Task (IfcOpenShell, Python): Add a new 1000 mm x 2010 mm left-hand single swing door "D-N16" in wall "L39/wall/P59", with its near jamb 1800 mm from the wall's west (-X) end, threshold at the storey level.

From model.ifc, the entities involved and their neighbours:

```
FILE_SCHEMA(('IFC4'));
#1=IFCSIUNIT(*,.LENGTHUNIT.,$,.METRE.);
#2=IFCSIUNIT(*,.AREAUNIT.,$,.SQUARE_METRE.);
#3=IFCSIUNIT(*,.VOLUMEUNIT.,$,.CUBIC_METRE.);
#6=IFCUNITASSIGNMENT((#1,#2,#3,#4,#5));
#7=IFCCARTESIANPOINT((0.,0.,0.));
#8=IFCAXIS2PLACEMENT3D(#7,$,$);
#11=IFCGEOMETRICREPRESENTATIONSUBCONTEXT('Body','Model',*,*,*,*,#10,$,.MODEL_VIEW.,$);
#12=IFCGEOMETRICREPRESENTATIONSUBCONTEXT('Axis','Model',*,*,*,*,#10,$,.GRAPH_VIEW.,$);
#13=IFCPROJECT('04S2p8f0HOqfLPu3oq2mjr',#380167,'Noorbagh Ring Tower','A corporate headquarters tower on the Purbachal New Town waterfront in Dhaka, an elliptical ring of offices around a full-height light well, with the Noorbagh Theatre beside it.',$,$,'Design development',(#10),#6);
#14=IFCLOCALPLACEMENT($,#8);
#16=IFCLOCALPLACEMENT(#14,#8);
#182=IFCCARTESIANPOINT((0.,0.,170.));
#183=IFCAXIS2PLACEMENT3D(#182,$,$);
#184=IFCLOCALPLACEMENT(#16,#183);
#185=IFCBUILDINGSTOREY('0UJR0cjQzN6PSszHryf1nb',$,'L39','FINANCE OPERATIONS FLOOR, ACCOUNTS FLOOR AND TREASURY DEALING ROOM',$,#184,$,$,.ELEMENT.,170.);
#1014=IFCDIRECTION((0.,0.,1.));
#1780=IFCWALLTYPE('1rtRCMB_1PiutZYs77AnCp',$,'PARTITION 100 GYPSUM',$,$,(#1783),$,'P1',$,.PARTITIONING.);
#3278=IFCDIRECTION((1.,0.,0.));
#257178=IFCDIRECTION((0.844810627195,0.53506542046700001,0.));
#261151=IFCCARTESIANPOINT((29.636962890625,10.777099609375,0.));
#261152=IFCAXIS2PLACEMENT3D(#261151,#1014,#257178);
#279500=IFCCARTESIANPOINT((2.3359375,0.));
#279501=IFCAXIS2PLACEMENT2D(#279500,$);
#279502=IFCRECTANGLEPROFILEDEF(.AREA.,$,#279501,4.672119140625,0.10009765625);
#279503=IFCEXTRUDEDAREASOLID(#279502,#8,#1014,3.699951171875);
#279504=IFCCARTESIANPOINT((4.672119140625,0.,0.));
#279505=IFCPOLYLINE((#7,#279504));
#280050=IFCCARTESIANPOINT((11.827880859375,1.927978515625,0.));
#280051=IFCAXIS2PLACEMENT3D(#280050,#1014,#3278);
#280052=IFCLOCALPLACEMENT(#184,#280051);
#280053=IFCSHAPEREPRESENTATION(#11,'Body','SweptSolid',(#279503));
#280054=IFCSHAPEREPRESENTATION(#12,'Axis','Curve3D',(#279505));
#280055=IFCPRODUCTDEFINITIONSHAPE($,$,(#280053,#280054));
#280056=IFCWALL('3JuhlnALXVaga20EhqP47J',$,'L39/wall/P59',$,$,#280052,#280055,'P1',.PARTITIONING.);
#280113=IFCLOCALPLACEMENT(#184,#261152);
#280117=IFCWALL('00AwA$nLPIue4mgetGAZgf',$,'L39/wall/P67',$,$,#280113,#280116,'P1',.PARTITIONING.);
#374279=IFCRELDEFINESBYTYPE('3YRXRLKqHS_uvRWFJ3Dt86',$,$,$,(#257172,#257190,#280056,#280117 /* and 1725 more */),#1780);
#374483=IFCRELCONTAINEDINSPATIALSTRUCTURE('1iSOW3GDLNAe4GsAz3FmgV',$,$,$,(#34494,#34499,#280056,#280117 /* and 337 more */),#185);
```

```python
import numpy as np
import ifcopenshell
import ifcopenshell.api.feature
import ifcopenshell.api.geometry
import ifcopenshell.api.root
import ifcopenshell.api.spatial
import ifcopenshell.geom
import ifcopenshell.util.element
import ifcopenshell.util.placement
import ifcopenshell.util.representation
import ifcopenshell.util.shape
import ifcopenshell.util.unit

model = ifcopenshell.open("model.ifc")
unit_scale = ifcopenshell.util.unit.calculate_unit_scale(model)
settings = ifcopenshell.geom.settings()


def volume(element):
    """Net volume in cubic metres, openings subtracted."""
    shape = ifcopenshell.geom.create_shape(settings, element)
    return ifcopenshell.util.shape.get_volume(shape.geometry)


wall = model.by_id(280056)
storey = ifcopenshell.util.element.get_container(wall, ifc_class="IfcBuildingStorey")
context = ifcopenshell.util.representation.get_context(model, "Model", "Body", "MODEL_VIEW")
before = volume(wall)

width, height, from_end, sill = 1, 2.01, 1.8, 0.0  # metres

# The wall runs along its own X axis, and the end named is its -X end.
wall_shape = ifcopenshell.geom.create_shape(settings, wall)
x, y, z = ifcopenshell.util.shape.get_vertices(wall_shape.geometry).T
start = x.min() + from_end
face, thickness = float(y.min()), float(y.max() - y.min())
wall_matrix = ifcopenshell.util.placement.get_local_placement(wall.ObjectPlacement)
level = ifcopenshell.util.placement.get_local_placement(storey.ObjectPlacement)[2, 3]


def in_wall(x, y):
    """Placement at x, y metres in the wall's axes, at sill height."""
    matrix = wall_matrix.copy()
    matrix[:, 3] = wall_matrix @ np.array([x / unit_scale, y / unit_scale, 0.0, 1.0])
    matrix[2, 3] = level + sill / unit_scale
    return matrix


# Opening: a box that overshoots both wall faces by 50 mm.
opening = ifcopenshell.api.root.create_entity(model, ifc_class="IfcOpeningElement", predefined_type="OPENING")
box = ifcopenshell.api.geometry.add_wall_representation(
    model, context=context, length=width, height=height, thickness=thickness + 0.1
)
ifcopenshell.api.geometry.assign_representation(model, product=opening, representation=box)
ifcopenshell.api.geometry.edit_object_placement(model, product=opening, matrix=in_wall(start, face - 0.05), is_si=False)
ifcopenshell.api.feature.add_feature(model, feature=opening, element=wall)

door = ifcopenshell.api.root.create_entity(model, ifc_class="IfcDoor", name="D-N16", predefined_type="DOOR")
door.OverallWidth, door.OverallHeight = width / unit_scale, height / unit_scale
door.OperationType = "SINGLE_SWING_LEFT"
body = ifcopenshell.api.geometry.add_door_representation(
    model,
    context=context,
    overall_width=door.OverallWidth,
    overall_height=door.OverallHeight,
    operation_type="SINGLE_SWING_LEFT",
    lining_properties={"LiningDepth": thickness / unit_scale, "ThresholdDepth": thickness / unit_scale},
)
ifcopenshell.api.geometry.assign_representation(model, product=door, representation=body)
ifcopenshell.api.spatial.assign_container(model, products=[door], relating_structure=storey)
ifcopenshell.api.feature.add_filling(model, opening=opening, element=door)

# The lining spans the wall, so the door starts at the wall face.
ifcopenshell.api.geometry.edit_object_placement(model, product=door, matrix=in_wall(start, face), is_si=False)

after = volume(wall)

print(f"wall volume {before:.3f} -> {after:.3f} m3")

model.write("model-out.ifc")
```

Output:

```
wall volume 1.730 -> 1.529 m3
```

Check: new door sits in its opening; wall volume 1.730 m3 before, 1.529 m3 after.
